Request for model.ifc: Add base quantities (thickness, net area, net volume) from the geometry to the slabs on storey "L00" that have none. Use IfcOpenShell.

First a look at what the model holds.

```python
import ifcopenshell
import ifcopenshell.util.element
import ifcopenshell.util.unit

model = ifcopenshell.open("model.ifc")
print(model.schema)
for unit_type in ("LENGTHUNIT", "AREAUNIT", "VOLUMEUNIT"):
    print(unit_type, ifcopenshell.util.unit.calculate_unit_scale(model, unit_type))
storey = next(s for s in model.by_type("IfcBuildingStorey") if s.Name == "L00")
slabs = [e for e in ifcopenshell.util.element.get_decomposition(storey) if e.is_a("IfcSlab")]
for e in sorted(slabs, key=lambda e: e.id()):
    print(e.id(), e.is_a(), e.Name, list(ifcopenshell.util.element.get_psets(e, qtos_only=True)), sep=" | ")
```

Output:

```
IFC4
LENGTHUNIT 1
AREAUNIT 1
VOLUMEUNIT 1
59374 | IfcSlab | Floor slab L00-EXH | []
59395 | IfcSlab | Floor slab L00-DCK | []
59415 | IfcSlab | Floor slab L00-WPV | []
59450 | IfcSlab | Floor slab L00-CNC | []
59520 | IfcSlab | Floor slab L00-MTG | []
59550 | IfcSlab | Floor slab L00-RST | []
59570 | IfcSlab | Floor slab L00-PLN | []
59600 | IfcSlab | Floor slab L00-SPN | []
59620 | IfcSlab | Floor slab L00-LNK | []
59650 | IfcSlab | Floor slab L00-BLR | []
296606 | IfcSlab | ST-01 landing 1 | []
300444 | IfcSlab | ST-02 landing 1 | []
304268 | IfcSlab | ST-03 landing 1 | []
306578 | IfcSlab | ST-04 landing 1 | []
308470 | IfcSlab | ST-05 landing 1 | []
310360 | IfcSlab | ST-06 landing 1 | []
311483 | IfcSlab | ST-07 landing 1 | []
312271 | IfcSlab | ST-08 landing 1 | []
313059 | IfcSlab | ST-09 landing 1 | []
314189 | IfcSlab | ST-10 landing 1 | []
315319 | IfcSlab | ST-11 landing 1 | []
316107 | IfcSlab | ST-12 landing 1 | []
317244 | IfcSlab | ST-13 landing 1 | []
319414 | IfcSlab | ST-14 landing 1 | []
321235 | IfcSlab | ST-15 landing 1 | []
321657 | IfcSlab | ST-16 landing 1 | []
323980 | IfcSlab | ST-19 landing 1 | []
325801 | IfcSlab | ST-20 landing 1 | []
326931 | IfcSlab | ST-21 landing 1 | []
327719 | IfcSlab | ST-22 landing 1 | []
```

```python
import ifcopenshell
import ifcopenshell.api.pset
import ifcopenshell.geom
import ifcopenshell.util.element
import ifcopenshell.util.shape
import ifcopenshell.util.unit

model = ifcopenshell.open("model.ifc")
unit_scale = ifcopenshell.util.unit.calculate_unit_scale(model)
area_scale = ifcopenshell.util.unit.calculate_unit_scale(model, "AREAUNIT")
volume_scale = ifcopenshell.util.unit.calculate_unit_scale(model, "VOLUMEUNIT")
settings = ifcopenshell.geom.settings()

storey = next(s for s in model.by_type("IfcBuildingStorey") if s.Name == "L00")
slabs = [e for e in ifcopenshell.util.element.get_decomposition(storey) if e.is_a("IfcSlab")]

for e in sorted(slabs, key=lambda e: e.id()):
    if ifcopenshell.util.element.get_psets(e, qtos_only=True, should_inherit=False):
        continue
    # Geometry comes back in metres, in the element's own axes.
    shape = ifcopenshell.geom.create_shape(settings, e)
    values = {
        "Width": ifcopenshell.util.shape.get_z(shape.geometry) / unit_scale,
        "NetArea": ifcopenshell.util.shape.get_footprint_area(shape.geometry) / area_scale,
        "NetVolume": ifcopenshell.util.shape.get_volume(shape.geometry) / volume_scale,
    }
    qto = ifcopenshell.api.pset.add_qto(model, product=e, name="Qto_SlabBaseQuantities")
    ifcopenshell.api.pset.edit_qto(model, qto=qto, properties=values)
    print(e.id(), {k: round(v, 3) for k, v in values.items()})

model.write("model_rev.ifc")
```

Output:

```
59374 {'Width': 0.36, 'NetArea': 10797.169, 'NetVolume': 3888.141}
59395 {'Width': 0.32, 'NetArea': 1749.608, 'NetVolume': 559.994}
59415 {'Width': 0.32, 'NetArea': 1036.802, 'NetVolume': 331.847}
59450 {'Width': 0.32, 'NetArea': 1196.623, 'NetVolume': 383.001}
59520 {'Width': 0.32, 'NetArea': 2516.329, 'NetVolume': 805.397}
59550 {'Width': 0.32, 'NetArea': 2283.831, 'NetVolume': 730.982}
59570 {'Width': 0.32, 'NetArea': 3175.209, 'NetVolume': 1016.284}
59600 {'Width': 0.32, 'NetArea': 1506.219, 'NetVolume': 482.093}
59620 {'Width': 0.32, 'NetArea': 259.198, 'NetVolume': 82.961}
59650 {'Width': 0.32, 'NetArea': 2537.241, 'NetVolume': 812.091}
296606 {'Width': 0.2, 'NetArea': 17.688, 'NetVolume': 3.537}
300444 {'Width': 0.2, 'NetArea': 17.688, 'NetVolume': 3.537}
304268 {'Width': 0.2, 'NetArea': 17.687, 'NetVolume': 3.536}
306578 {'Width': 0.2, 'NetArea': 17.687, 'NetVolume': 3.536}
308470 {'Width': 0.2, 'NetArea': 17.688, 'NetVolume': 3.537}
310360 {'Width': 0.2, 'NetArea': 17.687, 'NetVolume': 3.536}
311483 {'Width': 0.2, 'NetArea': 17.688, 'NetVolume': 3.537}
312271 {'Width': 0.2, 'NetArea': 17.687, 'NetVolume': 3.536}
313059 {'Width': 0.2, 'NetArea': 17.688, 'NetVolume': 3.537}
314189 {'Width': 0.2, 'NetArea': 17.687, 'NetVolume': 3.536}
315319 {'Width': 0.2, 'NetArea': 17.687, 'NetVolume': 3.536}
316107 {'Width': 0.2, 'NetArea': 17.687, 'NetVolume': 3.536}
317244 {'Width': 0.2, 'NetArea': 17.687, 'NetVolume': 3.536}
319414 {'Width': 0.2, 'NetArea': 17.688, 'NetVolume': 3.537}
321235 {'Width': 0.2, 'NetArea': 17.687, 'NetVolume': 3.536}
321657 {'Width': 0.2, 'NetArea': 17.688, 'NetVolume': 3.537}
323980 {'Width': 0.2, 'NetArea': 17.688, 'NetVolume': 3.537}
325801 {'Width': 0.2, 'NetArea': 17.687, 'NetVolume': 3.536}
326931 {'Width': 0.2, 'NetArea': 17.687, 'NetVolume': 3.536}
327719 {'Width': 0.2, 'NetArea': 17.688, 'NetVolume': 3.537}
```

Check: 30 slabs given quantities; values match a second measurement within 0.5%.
